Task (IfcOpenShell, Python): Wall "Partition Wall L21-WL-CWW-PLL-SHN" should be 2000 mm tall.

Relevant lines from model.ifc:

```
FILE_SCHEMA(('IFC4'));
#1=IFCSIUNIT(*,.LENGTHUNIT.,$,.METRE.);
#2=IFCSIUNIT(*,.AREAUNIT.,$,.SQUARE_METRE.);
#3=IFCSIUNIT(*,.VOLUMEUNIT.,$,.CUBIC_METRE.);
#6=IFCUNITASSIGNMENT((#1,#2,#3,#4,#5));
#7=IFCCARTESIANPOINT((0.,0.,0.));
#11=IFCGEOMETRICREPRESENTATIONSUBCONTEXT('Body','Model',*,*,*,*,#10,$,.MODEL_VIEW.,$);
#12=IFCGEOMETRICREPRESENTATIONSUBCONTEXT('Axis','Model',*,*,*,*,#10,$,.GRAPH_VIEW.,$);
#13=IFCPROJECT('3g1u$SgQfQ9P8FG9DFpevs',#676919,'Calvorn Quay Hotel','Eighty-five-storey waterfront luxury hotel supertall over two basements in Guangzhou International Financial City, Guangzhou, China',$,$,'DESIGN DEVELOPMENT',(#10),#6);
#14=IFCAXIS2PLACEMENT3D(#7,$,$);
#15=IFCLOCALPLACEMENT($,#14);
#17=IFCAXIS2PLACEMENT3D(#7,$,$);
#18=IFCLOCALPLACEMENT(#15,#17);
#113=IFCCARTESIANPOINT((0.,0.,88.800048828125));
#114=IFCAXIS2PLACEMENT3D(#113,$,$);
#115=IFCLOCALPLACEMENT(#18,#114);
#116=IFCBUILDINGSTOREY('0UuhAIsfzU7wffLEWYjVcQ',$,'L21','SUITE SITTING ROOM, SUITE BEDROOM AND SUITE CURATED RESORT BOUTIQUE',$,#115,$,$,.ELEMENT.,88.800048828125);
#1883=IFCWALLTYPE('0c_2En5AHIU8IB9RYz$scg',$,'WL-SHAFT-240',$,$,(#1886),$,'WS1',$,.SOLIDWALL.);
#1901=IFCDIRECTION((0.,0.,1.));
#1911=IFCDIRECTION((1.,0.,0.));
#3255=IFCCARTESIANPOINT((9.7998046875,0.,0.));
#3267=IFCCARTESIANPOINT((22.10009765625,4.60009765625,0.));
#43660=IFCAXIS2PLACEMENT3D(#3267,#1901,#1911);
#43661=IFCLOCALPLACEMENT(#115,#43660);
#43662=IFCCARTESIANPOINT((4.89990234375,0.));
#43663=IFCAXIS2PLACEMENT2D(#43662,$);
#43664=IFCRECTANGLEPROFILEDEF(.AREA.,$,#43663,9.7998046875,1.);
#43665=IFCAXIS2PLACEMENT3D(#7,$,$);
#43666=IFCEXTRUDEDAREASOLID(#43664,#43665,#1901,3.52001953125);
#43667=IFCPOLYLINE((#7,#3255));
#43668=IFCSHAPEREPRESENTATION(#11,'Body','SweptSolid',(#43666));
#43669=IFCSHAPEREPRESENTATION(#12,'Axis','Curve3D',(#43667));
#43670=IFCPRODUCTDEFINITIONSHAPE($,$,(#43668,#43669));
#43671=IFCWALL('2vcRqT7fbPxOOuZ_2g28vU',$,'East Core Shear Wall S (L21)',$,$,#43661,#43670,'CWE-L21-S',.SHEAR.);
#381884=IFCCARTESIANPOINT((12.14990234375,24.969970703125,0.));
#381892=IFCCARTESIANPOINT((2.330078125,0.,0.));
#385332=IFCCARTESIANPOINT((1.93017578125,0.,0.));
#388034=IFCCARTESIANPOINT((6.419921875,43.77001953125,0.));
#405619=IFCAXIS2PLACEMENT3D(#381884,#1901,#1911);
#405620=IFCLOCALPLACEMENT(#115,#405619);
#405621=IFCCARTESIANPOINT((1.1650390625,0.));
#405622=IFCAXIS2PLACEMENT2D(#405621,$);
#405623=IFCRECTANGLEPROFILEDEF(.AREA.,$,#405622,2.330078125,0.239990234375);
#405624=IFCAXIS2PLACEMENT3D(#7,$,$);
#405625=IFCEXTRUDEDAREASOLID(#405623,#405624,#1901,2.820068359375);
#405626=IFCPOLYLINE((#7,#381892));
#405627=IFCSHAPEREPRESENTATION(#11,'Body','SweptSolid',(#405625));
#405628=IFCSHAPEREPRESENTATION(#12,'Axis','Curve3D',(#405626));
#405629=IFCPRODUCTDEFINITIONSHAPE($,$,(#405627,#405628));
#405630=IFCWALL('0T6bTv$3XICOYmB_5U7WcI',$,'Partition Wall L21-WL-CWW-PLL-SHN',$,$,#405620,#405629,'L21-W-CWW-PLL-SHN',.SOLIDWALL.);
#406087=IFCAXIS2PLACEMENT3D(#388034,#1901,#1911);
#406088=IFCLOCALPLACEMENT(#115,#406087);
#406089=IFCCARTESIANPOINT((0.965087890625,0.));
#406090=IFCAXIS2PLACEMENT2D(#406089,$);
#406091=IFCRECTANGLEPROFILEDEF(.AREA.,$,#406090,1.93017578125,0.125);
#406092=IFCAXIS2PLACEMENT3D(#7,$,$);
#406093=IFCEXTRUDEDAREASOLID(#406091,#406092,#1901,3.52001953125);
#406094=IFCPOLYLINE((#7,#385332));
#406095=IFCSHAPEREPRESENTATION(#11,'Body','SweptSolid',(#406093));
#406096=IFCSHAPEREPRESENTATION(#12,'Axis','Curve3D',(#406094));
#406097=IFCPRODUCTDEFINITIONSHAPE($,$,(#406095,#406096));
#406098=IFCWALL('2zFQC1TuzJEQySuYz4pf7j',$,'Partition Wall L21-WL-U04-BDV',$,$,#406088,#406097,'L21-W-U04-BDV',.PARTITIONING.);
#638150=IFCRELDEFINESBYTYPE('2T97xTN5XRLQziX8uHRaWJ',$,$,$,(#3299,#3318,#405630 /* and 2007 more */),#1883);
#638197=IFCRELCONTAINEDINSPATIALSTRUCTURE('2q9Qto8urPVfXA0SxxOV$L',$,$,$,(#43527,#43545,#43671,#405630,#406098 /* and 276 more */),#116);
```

```python
import ifcopenshell
import ifcopenshell.geom
import ifcopenshell.util.representation
import ifcopenshell.util.shape
import ifcopenshell.util.unit

model = ifcopenshell.open("model.ifc")
unit_scale = ifcopenshell.util.unit.calculate_unit_scale(model)
settings = ifcopenshell.geom.settings()


def volume(element):
    """Net volume in cubic metres, openings subtracted."""
    shape = ifcopenshell.geom.create_shape(settings, element)
    return ifcopenshell.util.shape.get_volume(shape.geometry)


wall = model.by_guid("0T6bTv$3XICOYmB_5U7WcI")
before = volume(wall)

body = ifcopenshell.util.representation.get_representation(wall, "Model", "Body")
solid = body.Items[0]
old_height = solid.Depth
solid.Depth = 2 / unit_scale
after = volume(wall)

print(f"height {old_height:g} -> {solid.Depth:g}, volume {before:.3f} -> {after:.3f} m3")

model.write("model_edited.ifc")
```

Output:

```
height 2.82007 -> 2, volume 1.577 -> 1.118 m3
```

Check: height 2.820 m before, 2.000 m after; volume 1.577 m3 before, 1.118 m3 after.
